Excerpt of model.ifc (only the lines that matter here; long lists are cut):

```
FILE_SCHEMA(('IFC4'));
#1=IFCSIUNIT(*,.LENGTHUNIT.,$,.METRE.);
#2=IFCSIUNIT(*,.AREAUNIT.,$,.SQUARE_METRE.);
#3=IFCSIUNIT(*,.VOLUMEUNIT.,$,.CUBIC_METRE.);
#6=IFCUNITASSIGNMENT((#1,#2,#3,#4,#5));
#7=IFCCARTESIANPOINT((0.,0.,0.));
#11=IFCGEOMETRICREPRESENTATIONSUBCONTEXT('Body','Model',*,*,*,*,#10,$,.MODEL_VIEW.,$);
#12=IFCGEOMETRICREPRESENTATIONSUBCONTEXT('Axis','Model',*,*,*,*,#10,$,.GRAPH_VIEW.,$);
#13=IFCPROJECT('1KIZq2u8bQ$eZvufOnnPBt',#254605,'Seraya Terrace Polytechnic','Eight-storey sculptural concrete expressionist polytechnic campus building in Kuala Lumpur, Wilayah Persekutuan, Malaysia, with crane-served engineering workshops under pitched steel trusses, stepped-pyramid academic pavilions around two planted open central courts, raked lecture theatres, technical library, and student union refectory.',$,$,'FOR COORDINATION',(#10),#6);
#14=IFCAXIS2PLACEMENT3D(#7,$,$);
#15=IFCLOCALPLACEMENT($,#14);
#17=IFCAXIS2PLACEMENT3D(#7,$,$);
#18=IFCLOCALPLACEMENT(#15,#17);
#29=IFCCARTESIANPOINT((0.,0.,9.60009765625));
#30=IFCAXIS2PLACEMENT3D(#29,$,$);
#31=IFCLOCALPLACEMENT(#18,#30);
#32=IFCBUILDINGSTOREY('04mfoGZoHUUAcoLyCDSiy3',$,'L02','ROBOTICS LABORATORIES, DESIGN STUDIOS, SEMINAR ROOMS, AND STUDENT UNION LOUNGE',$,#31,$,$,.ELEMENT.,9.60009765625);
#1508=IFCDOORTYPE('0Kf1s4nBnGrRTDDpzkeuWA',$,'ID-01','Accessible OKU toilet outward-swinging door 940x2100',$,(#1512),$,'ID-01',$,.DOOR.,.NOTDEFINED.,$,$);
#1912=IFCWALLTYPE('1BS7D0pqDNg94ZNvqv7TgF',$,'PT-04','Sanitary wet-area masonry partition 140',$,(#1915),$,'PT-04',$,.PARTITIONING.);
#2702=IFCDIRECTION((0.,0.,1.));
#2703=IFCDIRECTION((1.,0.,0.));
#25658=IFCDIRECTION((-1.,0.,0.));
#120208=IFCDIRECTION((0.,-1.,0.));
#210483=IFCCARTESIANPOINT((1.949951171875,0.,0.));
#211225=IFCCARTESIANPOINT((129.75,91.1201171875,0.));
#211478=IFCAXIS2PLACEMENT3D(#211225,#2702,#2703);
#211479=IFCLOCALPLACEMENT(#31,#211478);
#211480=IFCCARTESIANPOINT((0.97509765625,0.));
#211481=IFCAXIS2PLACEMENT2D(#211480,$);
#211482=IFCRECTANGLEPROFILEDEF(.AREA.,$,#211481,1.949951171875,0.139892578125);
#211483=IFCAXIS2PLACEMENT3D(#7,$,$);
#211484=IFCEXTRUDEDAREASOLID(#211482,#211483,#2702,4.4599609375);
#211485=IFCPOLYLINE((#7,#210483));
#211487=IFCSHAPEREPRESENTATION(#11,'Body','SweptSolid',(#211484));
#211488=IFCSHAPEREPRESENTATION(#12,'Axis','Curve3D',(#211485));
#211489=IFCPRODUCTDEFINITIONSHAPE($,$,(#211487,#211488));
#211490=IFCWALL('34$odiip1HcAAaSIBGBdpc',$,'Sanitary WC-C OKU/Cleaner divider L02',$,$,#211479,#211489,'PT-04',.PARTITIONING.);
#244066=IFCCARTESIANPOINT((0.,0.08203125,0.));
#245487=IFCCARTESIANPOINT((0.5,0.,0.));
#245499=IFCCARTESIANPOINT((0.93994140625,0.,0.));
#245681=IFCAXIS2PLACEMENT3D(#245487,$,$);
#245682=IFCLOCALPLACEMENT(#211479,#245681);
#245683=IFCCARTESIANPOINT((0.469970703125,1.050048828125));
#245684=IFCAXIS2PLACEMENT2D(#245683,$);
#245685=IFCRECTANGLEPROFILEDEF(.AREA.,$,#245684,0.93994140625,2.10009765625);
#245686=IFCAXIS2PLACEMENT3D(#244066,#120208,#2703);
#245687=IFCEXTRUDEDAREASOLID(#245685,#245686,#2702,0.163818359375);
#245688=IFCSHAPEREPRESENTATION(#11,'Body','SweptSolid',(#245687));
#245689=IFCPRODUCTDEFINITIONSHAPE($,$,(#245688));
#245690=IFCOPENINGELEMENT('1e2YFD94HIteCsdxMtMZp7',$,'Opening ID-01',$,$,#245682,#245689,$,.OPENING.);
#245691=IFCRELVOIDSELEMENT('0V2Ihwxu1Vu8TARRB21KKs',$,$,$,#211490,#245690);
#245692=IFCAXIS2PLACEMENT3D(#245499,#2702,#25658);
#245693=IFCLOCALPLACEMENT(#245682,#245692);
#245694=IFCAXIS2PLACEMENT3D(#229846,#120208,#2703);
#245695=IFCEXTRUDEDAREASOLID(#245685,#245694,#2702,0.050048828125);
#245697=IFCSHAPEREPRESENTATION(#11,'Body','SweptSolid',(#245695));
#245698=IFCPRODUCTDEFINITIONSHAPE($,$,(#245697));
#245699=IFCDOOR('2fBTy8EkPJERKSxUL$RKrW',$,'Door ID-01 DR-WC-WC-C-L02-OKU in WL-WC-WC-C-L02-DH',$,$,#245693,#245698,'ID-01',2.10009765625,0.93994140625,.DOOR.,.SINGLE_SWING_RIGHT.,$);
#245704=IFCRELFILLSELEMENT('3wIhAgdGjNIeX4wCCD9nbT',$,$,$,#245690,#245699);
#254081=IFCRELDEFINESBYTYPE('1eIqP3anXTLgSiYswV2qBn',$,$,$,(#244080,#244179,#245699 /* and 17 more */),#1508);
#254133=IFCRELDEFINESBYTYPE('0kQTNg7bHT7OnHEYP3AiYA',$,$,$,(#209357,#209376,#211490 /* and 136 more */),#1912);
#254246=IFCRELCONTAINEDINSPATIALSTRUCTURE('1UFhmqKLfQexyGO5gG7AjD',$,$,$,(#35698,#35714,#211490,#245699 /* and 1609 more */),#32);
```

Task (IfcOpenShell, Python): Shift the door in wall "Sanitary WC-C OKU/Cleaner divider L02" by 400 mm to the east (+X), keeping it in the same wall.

```python
import ifcopenshell
import ifcopenshell.api.geometry
import ifcopenshell.util.placement

model = ifcopenshell.open("model.ifc")

door = model.by_id(245699)
opening = door.FillsVoids[0].RelatingOpeningElement
wall = opening.VoidsElements[0].RelatingBuildingElement

wall_matrix = ifcopenshell.util.placement.get_local_placement(wall.ObjectPlacement)
shift = wall_matrix[:3, 0] * 0.4
before = ifcopenshell.util.placement.get_local_placement(door.ObjectPlacement)[:3, 3].copy()

# The door is placed relative to its opening, so it follows when the opening moves.
matrix = ifcopenshell.util.placement.get_local_placement(opening.ObjectPlacement)
matrix[:3, 3] += shift
ifcopenshell.api.geometry.edit_object_placement(
    model, product=opening, matrix=matrix, is_si=False, should_transform_children=True
)

after = ifcopenshell.util.placement.get_local_placement(door.ObjectPlacement)[:3, 3]
print("door moved by", (after - before).round(3) + 0.0)

model.write("model_v2.ifc")
```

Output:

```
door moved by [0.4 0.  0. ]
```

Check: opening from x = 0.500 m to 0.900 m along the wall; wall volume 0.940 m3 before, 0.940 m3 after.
